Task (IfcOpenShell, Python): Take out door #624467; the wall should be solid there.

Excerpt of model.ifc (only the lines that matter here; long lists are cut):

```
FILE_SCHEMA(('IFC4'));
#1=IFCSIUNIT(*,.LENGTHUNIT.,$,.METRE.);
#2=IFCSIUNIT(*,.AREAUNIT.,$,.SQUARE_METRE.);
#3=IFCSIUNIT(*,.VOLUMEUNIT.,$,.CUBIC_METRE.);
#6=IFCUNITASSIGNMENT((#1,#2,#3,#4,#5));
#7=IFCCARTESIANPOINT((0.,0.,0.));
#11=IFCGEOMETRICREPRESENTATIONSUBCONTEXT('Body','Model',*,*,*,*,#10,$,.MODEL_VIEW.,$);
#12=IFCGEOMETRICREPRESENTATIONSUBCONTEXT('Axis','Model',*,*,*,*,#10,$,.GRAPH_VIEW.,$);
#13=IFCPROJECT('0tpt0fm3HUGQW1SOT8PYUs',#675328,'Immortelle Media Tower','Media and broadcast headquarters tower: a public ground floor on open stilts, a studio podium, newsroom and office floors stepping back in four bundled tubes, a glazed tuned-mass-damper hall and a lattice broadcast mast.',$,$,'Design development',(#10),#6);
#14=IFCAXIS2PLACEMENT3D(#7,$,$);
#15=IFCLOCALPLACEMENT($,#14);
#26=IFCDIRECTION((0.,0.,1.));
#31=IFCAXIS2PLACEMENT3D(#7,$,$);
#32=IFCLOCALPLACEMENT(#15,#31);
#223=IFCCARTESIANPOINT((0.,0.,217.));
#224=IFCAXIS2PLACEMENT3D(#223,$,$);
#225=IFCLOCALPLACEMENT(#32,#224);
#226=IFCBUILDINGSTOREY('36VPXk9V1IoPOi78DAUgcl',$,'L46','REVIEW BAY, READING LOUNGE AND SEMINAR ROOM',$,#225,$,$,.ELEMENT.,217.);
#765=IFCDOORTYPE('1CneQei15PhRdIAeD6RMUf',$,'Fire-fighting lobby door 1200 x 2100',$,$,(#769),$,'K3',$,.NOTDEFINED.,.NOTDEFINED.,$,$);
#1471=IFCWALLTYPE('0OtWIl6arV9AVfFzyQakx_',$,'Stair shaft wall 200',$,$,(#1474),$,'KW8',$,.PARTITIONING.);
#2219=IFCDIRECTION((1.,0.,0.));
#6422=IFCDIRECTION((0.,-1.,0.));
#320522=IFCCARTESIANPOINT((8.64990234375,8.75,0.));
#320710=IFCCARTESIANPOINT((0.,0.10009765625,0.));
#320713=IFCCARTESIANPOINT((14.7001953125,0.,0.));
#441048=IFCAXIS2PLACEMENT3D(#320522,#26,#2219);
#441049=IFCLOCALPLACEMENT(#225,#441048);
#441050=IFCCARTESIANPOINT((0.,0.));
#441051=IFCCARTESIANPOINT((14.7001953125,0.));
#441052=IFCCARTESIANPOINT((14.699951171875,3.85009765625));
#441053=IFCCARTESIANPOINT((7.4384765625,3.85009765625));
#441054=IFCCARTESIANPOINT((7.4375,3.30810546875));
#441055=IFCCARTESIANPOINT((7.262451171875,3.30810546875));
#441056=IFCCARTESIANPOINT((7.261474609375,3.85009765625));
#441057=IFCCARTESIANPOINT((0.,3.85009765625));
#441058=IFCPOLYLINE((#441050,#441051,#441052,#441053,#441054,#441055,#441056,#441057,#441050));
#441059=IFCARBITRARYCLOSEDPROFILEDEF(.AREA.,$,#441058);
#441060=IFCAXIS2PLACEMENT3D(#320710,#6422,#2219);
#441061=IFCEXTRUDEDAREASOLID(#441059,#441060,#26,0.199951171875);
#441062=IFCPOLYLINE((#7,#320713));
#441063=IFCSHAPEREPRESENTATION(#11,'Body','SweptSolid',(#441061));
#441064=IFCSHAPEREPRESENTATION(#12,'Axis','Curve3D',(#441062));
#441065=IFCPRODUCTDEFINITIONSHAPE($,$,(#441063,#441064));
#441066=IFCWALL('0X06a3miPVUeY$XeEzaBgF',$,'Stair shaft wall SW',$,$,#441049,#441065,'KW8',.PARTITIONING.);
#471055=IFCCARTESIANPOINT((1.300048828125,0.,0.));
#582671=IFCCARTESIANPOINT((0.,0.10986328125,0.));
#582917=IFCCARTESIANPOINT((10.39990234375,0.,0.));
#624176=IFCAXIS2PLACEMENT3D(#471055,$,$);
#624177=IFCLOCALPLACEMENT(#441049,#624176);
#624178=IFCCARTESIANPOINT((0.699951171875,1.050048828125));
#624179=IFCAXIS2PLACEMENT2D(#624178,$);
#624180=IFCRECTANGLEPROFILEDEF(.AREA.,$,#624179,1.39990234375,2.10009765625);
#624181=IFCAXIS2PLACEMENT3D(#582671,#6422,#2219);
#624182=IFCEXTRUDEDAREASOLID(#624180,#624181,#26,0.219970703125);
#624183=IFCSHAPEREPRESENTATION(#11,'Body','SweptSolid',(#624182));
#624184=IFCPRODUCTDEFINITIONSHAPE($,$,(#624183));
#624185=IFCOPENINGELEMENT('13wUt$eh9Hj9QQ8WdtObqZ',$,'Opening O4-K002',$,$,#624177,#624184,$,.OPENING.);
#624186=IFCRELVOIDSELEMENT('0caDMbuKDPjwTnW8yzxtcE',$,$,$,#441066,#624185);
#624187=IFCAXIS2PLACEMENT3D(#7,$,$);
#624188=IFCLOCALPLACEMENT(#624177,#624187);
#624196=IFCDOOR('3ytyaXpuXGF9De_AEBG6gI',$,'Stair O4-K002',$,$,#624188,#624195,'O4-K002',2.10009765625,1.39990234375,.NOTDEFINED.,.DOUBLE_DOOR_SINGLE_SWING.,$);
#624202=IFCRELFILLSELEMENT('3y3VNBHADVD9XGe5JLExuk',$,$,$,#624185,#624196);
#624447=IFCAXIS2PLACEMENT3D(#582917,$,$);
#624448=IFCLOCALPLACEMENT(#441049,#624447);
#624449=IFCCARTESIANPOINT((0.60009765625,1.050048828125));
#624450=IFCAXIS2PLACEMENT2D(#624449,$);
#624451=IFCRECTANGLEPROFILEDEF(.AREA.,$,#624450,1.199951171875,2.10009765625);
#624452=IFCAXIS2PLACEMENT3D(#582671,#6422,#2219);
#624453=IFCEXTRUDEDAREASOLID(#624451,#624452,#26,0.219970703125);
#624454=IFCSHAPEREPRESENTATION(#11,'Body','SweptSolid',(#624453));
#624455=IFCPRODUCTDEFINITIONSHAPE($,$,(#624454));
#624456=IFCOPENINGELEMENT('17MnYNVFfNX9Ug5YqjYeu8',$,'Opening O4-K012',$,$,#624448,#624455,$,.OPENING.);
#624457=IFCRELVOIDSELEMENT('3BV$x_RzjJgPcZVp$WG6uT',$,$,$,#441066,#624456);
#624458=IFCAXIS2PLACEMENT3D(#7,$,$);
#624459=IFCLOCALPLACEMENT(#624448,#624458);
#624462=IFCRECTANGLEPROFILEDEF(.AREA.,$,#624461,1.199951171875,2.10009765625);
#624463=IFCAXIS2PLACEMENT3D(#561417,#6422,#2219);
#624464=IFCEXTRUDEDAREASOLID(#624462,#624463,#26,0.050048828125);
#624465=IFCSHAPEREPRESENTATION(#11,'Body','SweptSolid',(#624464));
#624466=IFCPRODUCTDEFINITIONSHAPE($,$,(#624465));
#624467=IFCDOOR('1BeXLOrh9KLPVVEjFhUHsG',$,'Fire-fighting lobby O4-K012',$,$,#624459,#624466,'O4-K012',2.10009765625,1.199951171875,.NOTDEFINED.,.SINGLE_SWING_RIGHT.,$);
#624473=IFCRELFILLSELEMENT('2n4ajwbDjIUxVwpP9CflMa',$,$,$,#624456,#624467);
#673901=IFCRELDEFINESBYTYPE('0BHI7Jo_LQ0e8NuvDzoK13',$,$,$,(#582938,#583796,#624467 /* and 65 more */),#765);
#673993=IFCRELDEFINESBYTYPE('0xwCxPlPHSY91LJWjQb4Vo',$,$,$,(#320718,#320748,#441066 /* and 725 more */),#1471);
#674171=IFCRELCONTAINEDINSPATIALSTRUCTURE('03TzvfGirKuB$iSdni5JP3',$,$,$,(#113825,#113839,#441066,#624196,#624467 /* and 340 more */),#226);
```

```python
import ifcopenshell
import ifcopenshell.api.feature
import ifcopenshell.api.root
import ifcopenshell.geom
import ifcopenshell.util.shape

model = ifcopenshell.open("model.ifc")
settings = ifcopenshell.geom.settings()


def volume(element):
    """Net volume in cubic metres, openings subtracted."""
    shape = ifcopenshell.geom.create_shape(settings, element)
    return ifcopenshell.util.shape.get_volume(shape.geometry)


door = model.by_guid("1BeXLOrh9KLPVVEjFhUHsG")
opening = door.FillsVoids[0].RelatingOpeningElement
wall = opening.VoidsElements[0].RelatingBuildingElement
before = volume(wall)

ifcopenshell.api.root.remove_product(model, product=door)
ifcopenshell.api.feature.remove_feature(model, feature=opening)

after = volume(wall)

print(f"wall volume {before:.3f} -> {after:.3f} m3")

model.write("model_rev.ifc")
```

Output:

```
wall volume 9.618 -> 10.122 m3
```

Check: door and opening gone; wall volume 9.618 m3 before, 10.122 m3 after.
